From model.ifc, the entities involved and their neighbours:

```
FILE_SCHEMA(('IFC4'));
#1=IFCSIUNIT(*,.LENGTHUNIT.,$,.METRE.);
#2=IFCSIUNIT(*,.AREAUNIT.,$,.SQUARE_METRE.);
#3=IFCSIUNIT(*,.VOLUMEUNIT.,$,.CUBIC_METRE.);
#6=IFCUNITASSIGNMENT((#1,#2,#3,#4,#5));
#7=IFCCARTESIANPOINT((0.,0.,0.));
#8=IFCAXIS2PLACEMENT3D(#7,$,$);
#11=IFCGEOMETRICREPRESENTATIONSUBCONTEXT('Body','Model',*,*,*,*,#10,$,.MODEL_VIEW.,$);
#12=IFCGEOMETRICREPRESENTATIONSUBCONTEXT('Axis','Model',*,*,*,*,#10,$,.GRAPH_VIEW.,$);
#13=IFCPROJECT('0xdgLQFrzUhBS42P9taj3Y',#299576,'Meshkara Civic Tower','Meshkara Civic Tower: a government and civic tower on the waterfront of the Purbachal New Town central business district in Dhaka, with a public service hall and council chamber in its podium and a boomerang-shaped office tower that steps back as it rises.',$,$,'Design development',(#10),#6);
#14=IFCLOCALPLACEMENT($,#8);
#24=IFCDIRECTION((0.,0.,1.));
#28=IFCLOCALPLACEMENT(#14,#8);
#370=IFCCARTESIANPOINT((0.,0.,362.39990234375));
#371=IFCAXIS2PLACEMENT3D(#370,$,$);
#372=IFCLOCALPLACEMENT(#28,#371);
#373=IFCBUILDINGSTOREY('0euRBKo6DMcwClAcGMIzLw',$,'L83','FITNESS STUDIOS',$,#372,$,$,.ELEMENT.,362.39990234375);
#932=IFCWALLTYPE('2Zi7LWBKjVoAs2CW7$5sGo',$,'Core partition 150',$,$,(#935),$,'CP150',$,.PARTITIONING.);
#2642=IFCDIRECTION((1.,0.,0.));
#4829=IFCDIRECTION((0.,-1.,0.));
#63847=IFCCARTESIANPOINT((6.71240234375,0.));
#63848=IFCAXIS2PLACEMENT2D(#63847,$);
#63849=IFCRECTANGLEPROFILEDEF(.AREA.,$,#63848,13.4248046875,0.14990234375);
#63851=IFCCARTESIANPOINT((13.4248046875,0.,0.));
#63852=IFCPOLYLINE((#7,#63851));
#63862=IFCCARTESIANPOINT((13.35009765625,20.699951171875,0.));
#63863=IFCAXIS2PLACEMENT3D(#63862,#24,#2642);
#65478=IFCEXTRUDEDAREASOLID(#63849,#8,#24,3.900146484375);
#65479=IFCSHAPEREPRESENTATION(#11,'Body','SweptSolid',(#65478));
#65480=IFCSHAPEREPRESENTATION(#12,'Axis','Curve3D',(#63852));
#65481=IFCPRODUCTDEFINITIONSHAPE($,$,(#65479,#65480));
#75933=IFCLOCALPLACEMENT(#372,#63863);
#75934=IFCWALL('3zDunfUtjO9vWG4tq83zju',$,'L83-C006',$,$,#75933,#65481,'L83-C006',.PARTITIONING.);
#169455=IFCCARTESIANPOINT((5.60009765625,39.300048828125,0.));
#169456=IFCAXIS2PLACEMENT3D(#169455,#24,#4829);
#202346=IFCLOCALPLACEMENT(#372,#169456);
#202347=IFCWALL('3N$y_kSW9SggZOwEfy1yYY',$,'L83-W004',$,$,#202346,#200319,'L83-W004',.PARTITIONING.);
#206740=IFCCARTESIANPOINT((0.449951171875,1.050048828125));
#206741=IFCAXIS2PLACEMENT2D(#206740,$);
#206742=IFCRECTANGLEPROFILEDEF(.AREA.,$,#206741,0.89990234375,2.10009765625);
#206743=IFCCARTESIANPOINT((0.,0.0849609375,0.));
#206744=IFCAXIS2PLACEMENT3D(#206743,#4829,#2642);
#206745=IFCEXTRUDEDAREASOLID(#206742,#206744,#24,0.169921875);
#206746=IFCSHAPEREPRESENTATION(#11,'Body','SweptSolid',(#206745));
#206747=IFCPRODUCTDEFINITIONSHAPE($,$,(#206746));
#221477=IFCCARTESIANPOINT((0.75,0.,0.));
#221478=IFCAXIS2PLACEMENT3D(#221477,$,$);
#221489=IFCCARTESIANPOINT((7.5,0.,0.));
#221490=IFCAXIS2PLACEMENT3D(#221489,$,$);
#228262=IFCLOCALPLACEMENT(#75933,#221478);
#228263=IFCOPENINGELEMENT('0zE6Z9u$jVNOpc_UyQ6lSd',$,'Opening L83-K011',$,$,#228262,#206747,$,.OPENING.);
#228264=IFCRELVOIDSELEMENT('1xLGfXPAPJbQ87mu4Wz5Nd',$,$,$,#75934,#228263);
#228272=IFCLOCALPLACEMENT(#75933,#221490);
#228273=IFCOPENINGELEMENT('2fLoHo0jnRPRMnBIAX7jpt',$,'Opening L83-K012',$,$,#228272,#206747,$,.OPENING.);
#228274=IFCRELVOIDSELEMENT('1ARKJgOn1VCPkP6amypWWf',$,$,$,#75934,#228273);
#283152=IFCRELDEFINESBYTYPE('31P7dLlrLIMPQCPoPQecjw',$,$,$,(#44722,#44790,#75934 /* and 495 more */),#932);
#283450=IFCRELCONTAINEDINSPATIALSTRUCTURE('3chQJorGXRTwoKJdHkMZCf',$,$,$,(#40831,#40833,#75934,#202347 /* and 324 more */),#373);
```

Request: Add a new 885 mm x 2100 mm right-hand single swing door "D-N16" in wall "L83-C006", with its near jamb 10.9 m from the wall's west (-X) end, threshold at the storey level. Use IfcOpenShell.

```python
import numpy as np
import ifcopenshell
import ifcopenshell.api.feature
import ifcopenshell.api.geometry
import ifcopenshell.api.root
import ifcopenshell.api.spatial
import ifcopenshell.geom
import ifcopenshell.util.element
import ifcopenshell.util.placement
import ifcopenshell.util.representation
import ifcopenshell.util.shape
import ifcopenshell.util.unit

model = ifcopenshell.open("model.ifc")
unit_scale = ifcopenshell.util.unit.calculate_unit_scale(model)
settings = ifcopenshell.geom.settings()


def volume(element):
    """Net volume in cubic metres, openings subtracted."""
    shape = ifcopenshell.geom.create_shape(settings, element)
    return ifcopenshell.util.shape.get_volume(shape.geometry)


wall = model.by_id(75934)
storey = ifcopenshell.util.element.get_container(wall, ifc_class="IfcBuildingStorey")
context = ifcopenshell.util.representation.get_context(model, "Model", "Body", "MODEL_VIEW")
before = volume(wall)

width, height, from_end, sill = 0.885, 2.1, 10.9, 0.0  # metres

# The wall runs along its own X axis, and the end named is its -X end.
wall_shape = ifcopenshell.geom.create_shape(settings, wall)
x, y, z = ifcopenshell.util.shape.get_vertices(wall_shape.geometry).T
start = x.min() + from_end
face, thickness = float(y.min()), float(y.max() - y.min())
wall_matrix = ifcopenshell.util.placement.get_local_placement(wall.ObjectPlacement)
level = ifcopenshell.util.placement.get_local_placement(storey.ObjectPlacement)[2, 3]


def in_wall(x, y):
    """Placement at x, y metres in the wall's axes, at sill height."""
    matrix = wall_matrix.copy()
    matrix[:, 3] = wall_matrix @ np.array([x / unit_scale, y / unit_scale, 0.0, 1.0])
    matrix[2, 3] = level + sill / unit_scale
    return matrix


# Opening: a box that overshoots both wall faces by 50 mm.
opening = ifcopenshell.api.root.create_entity(model, ifc_class="IfcOpeningElement", predefined_type="OPENING")
box = ifcopenshell.api.geometry.add_wall_representation(
    model, context=context, length=width, height=height, thickness=thickness + 0.1
)
ifcopenshell.api.geometry.assign_representation(model, product=opening, representation=box)
ifcopenshell.api.geometry.edit_object_placement(model, product=opening, matrix=in_wall(start, face - 0.05), is_si=False)
ifcopenshell.api.feature.add_feature(model, feature=opening, element=wall)

door = ifcopenshell.api.root.create_entity(model, ifc_class="IfcDoor", name="D-N16", predefined_type="DOOR")
door.OverallWidth, door.OverallHeight = width / unit_scale, height / unit_scale
door.OperationType = "SINGLE_SWING_RIGHT"
body = ifcopenshell.api.geometry.add_door_representation(
    model,
    context=context,
    overall_width=door.OverallWidth,
    overall_height=door.OverallHeight,
    operation_type="SINGLE_SWING_RIGHT",
    lining_properties={"LiningDepth": thickness / unit_scale, "ThresholdDepth": thickness / unit_scale},
)
ifcopenshell.api.geometry.assign_representation(model, product=door, representation=body)
ifcopenshell.api.spatial.assign_container(model, products=[door], relating_structure=storey)
ifcopenshell.api.feature.add_filling(model, opening=opening, element=door)

# The lining spans the wall, so the door starts at the wall face.
ifcopenshell.api.geometry.edit_object_placement(model, product=door, matrix=in_wall(start, face), is_si=False)

after = volume(wall)

print(f"wall volume {before:.3f} -> {after:.3f} m3")

model.write("model-out.ifc")
```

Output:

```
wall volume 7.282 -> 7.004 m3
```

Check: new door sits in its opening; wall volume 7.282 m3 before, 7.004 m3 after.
